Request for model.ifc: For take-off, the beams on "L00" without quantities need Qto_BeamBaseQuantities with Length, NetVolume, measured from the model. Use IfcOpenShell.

First a look at what the model holds.

```python
import ifcopenshell
import ifcopenshell.util.element
import ifcopenshell.util.unit

model = ifcopenshell.open("model.ifc")
print(model.schema)
for unit_type in ("LENGTHUNIT", "AREAUNIT", "VOLUMEUNIT"):
    print(unit_type, ifcopenshell.util.unit.calculate_unit_scale(model, unit_type))
storey = next(s for s in model.by_type("IfcBuildingStorey") if s.Name == "L00")
beams = [e for e in ifcopenshell.util.element.get_decomposition(storey) if e.is_a("IfcBeam")]
for e in sorted(beams, key=lambda e: e.id()):
    print(e.id(), e.is_a(), e.Name, list(ifcopenshell.util.element.get_psets(e, qtos_only=True)), sep=" | ")
```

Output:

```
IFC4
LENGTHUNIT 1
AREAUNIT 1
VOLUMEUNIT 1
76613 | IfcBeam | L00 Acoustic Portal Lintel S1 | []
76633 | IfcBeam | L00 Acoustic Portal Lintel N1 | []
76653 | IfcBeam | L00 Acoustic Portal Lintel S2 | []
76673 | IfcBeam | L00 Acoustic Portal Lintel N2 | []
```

```python
import ifcopenshell
import ifcopenshell.api.pset
import ifcopenshell.geom
import ifcopenshell.util.element
import ifcopenshell.util.shape
import ifcopenshell.util.unit

model = ifcopenshell.open("model.ifc")
unit_scale = ifcopenshell.util.unit.calculate_unit_scale(model)
volume_scale = ifcopenshell.util.unit.calculate_unit_scale(model, "VOLUMEUNIT")
settings = ifcopenshell.geom.settings()

storey = next(s for s in model.by_type("IfcBuildingStorey") if s.Name == "L00")
beams = [e for e in ifcopenshell.util.element.get_decomposition(storey) if e.is_a("IfcBeam")]

for e in sorted(beams, key=lambda e: e.id()):
    if ifcopenshell.util.element.get_psets(e, qtos_only=True, should_inherit=False):
        continue
    # Geometry comes back in metres, in the element's own axes.
    shape = ifcopenshell.geom.create_shape(settings, e)
    values = {
        "Length": ifcopenshell.util.shape.get_max_xyz(shape.geometry) / unit_scale,
        "NetVolume": ifcopenshell.util.shape.get_volume(shape.geometry) / volume_scale,
    }
    qto = ifcopenshell.api.pset.add_qto(model, product=e, name="Qto_BeamBaseQuantities")
    ifcopenshell.api.pset.edit_qto(model, qto=qto, properties=values)
    print(e.id(), {k: round(v, 3) for k, v in values.items()})

model.write("model_edited.ifc")
```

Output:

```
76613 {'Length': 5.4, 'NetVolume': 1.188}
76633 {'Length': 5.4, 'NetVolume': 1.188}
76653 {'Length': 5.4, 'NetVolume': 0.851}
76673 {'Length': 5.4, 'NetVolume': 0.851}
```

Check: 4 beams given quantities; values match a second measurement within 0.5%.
